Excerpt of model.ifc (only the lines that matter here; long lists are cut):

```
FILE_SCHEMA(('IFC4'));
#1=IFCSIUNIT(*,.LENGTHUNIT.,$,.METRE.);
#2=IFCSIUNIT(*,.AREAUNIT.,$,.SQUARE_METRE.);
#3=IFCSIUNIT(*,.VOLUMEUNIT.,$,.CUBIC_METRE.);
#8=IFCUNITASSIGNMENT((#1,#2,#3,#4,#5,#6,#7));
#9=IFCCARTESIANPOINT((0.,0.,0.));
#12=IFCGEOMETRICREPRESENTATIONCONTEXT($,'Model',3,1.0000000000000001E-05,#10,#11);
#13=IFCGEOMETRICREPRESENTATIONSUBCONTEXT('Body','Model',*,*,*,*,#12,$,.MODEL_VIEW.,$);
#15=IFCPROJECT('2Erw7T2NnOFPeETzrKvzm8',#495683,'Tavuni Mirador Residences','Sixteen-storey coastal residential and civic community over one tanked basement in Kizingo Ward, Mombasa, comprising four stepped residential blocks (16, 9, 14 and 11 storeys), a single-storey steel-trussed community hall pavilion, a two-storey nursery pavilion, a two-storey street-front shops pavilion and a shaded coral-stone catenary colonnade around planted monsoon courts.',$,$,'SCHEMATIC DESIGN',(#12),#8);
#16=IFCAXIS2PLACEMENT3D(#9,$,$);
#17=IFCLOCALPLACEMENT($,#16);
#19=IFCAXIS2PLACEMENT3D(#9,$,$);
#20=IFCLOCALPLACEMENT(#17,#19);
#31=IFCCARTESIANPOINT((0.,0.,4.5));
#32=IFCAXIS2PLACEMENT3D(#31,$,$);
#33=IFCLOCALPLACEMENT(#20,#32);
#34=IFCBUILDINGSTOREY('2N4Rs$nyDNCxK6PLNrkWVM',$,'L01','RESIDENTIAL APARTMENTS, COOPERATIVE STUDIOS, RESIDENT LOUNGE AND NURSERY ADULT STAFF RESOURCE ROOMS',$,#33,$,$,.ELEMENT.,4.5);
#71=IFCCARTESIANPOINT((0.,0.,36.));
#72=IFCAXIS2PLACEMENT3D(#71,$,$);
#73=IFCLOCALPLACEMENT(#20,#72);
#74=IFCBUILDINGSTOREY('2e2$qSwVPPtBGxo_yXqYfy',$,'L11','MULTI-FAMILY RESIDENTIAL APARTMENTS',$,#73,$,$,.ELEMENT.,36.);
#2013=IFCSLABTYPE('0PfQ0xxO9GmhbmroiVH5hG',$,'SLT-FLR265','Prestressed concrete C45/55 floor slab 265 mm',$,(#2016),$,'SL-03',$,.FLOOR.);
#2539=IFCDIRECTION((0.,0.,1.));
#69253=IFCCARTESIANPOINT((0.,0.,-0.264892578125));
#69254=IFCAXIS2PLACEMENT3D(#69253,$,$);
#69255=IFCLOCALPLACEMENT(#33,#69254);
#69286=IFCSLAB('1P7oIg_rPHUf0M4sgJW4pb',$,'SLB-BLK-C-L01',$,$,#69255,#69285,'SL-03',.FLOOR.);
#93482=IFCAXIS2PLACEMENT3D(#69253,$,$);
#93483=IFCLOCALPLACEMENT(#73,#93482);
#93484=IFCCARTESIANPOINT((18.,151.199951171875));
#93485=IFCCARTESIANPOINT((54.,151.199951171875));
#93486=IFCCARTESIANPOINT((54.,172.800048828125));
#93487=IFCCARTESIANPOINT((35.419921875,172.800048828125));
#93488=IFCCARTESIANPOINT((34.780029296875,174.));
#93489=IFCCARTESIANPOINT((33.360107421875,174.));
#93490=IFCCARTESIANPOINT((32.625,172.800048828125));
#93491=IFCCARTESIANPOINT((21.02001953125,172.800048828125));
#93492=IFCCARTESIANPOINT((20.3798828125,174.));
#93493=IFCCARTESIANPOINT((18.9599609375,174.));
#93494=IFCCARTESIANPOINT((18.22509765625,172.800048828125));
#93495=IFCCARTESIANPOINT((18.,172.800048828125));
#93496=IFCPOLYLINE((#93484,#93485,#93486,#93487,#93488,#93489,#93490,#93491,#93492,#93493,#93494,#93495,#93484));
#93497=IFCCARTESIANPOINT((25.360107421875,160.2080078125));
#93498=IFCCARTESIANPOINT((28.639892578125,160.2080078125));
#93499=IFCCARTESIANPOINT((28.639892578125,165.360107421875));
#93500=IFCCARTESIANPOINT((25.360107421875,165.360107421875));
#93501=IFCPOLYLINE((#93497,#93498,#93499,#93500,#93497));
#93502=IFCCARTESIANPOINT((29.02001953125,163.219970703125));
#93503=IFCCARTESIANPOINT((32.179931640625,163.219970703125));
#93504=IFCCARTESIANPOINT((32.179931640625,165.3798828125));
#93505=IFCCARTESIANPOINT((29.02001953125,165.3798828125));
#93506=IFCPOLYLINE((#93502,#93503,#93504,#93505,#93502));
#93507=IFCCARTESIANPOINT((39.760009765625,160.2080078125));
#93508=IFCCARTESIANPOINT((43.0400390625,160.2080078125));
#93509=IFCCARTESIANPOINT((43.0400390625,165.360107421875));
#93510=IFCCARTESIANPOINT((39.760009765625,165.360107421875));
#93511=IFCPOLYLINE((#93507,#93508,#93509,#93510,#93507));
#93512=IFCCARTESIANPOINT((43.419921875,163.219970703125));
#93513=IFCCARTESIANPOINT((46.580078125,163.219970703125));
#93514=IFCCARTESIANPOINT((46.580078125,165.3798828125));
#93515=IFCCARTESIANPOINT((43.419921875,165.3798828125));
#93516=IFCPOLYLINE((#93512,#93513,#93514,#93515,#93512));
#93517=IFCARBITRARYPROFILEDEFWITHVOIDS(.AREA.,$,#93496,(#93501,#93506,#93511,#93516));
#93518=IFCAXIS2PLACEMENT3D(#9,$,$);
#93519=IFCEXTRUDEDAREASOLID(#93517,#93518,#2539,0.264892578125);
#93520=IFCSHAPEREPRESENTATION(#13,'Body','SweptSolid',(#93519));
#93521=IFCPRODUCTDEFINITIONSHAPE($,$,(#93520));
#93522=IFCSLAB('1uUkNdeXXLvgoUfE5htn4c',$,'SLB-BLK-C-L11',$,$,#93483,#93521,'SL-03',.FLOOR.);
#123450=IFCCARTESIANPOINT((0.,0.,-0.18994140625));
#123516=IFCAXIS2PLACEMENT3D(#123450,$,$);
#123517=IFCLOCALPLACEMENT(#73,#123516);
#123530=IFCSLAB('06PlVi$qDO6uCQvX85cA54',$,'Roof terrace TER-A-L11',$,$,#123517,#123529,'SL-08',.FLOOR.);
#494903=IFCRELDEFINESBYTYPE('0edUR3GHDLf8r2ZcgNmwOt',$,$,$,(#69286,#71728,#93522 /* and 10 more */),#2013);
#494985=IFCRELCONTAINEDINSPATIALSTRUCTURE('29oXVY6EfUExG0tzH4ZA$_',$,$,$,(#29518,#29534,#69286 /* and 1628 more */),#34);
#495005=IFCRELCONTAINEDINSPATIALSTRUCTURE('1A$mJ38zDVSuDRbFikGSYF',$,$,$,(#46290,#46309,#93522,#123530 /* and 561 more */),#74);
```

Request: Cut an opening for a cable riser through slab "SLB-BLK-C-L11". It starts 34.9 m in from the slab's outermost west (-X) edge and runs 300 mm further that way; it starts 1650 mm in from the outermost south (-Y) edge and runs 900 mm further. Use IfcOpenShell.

```python
import numpy as np
import ifcopenshell
import ifcopenshell.api.feature
import ifcopenshell.api.geometry
import ifcopenshell.api.root
import ifcopenshell.geom
import ifcopenshell.util.placement
import ifcopenshell.util.representation
import ifcopenshell.util.shape
import ifcopenshell.util.unit

model = ifcopenshell.open("model.ifc")
unit_scale = ifcopenshell.util.unit.calculate_unit_scale(model)
settings = ifcopenshell.geom.settings()


def volume(element):
    """Net volume in cubic metres, openings subtracted."""
    shape = ifcopenshell.geom.create_shape(settings, element)
    return ifcopenshell.util.shape.get_volume(shape.geometry)


slab = model.by_guid("1uUkNdeXXLvgoUfE5htn4c")
before = volume(slab)

# Extent in the slab's own axes, in metres. The edges named are its -X and -Y sides.
slab_shape = ifcopenshell.geom.create_shape(settings, slab)
vertices = ifcopenshell.util.shape.get_vertices(slab_shape.geometry)
x_min, y_min, bottom = vertices.min(axis=0)
top = vertices[:, 2].max()

opening = ifcopenshell.api.root.create_entity(model, ifc_class="IfcOpeningElement", name="Cable riser opening", predefined_type="OPENING")
context = ifcopenshell.util.representation.get_context(model, "Model", "Body", "MODEL_VIEW")
width, depth = 0.3, 0.9
outline = [(0.0, 0.0), (width, 0.0), (width, depth), (0.0, depth), (0.0, 0.0)]
# Overshoot both faces by 50 mm so the cut is clean.
shape = ifcopenshell.api.geometry.add_slab_representation(
    model, context=context, depth=top - bottom + 0.1, polyline=outline
)
ifcopenshell.api.geometry.assign_representation(model, product=opening, representation=shape)

matrix = ifcopenshell.util.placement.get_local_placement(slab.ObjectPlacement)
matrix[:, 3] = matrix @ np.append(np.array([x_min + 34.9, y_min + 1.65, bottom - 0.05]) / unit_scale, 1.0)
ifcopenshell.api.geometry.edit_object_placement(model, product=opening, matrix=matrix, is_si=False)
ifcopenshell.api.feature.add_feature(model, feature=opening, element=slab)

after = volume(slab)

print(f"slab volume {before:.3f} -> {after:.3f} m3")

model.write("model_updated.ifc")
```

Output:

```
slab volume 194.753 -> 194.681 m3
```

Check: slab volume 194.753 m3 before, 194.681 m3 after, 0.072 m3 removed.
